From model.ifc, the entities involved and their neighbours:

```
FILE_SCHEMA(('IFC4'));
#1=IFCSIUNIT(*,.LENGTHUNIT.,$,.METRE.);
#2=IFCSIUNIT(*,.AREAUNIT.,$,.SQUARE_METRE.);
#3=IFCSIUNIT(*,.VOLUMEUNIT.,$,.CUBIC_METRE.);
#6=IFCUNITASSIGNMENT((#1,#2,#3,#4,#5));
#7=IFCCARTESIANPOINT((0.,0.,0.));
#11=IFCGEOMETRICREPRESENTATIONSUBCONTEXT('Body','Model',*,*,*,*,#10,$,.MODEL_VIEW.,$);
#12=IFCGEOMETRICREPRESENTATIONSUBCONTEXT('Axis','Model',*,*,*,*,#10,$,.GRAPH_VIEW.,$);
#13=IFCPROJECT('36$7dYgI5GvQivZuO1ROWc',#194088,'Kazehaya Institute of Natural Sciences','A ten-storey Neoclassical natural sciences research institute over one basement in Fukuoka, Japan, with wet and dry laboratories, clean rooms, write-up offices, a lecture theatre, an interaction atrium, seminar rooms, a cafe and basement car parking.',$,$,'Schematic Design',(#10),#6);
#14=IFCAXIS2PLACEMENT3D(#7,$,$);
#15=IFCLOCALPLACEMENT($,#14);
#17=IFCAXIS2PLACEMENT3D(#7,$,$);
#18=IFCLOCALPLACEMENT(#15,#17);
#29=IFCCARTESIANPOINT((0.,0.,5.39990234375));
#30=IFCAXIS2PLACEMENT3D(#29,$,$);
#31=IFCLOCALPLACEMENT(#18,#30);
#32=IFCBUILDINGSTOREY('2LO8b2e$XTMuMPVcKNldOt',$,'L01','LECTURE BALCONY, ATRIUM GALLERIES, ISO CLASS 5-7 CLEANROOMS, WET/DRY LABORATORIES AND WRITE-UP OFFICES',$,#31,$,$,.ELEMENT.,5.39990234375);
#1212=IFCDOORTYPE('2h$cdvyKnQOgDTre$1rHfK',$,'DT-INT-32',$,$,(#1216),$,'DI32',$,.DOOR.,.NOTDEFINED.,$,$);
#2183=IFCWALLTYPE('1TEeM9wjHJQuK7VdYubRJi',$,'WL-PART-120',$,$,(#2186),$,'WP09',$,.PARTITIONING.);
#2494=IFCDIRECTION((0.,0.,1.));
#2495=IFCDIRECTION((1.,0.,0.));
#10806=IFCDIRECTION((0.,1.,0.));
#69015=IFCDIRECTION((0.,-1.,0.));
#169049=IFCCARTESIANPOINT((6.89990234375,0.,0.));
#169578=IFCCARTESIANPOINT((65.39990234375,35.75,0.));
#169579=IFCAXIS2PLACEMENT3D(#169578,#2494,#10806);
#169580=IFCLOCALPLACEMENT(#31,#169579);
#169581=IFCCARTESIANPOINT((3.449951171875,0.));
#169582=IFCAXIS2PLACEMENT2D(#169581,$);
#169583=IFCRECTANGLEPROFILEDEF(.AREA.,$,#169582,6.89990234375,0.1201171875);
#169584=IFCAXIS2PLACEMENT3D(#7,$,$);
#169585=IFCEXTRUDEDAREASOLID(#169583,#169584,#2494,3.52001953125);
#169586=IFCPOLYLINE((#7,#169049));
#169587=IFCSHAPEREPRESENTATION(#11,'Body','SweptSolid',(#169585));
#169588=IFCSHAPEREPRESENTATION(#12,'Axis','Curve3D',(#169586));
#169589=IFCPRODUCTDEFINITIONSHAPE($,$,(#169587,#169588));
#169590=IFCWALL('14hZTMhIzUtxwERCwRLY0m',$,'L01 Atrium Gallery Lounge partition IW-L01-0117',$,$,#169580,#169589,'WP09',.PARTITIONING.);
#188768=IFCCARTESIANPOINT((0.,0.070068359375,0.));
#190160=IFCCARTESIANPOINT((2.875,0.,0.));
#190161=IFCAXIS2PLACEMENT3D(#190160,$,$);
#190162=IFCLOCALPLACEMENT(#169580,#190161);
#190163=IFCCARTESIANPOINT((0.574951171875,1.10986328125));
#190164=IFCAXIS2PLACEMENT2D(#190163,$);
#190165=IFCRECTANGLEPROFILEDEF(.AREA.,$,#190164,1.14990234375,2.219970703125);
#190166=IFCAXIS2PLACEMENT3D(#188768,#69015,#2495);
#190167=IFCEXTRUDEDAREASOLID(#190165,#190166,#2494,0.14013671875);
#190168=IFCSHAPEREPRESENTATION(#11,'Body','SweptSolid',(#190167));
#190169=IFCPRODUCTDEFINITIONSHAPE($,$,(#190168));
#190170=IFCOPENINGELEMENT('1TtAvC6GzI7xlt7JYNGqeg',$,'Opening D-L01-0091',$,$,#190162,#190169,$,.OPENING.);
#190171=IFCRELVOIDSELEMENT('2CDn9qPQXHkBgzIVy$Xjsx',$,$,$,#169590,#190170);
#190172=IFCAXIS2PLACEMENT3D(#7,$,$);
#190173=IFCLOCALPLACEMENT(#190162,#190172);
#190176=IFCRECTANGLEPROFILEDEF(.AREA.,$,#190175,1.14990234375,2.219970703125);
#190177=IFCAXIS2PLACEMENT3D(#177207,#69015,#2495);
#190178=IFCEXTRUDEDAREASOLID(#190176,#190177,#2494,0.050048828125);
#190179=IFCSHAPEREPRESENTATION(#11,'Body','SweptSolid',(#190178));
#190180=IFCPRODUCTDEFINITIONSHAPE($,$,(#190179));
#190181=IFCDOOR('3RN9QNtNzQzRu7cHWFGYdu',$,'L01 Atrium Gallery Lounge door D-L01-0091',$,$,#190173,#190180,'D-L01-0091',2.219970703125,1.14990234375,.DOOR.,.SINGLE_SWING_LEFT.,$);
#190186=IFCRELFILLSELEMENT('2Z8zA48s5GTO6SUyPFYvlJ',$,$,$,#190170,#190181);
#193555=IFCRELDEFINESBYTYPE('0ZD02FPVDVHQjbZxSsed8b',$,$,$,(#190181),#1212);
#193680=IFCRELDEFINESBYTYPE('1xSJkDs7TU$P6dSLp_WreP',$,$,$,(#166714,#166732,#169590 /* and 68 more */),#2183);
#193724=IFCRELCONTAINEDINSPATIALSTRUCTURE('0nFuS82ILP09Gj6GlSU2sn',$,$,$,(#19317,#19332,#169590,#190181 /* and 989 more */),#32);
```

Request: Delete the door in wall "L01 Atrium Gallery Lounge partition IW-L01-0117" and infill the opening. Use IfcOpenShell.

```python
import ifcopenshell
import ifcopenshell.api.feature
import ifcopenshell.api.root
import ifcopenshell.geom
import ifcopenshell.util.shape

model = ifcopenshell.open("model.ifc")
settings = ifcopenshell.geom.settings()


def volume(element):
    """Net volume in cubic metres, openings subtracted."""
    shape = ifcopenshell.geom.create_shape(settings, element)
    return ifcopenshell.util.shape.get_volume(shape.geometry)


door = model.by_guid("3RN9QNtNzQzRu7cHWFGYdu")
opening = door.FillsVoids[0].RelatingOpeningElement
wall = opening.VoidsElements[0].RelatingBuildingElement
before = volume(wall)

ifcopenshell.api.root.remove_product(model, product=door)
ifcopenshell.api.feature.remove_feature(model, feature=opening)

after = volume(wall)

print(f"wall volume {before:.3f} -> {after:.3f} m3")

model.write("model_v2.ifc")
```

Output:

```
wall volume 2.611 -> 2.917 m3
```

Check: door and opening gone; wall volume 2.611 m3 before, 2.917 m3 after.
